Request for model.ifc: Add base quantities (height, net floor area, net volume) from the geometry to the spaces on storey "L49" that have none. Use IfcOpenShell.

First a look at what the model holds.

```python
import ifcopenshell
import ifcopenshell.util.element
import ifcopenshell.util.unit

model = ifcopenshell.open("model.ifc")
print(model.schema)
for unit_type in ("LENGTHUNIT", "AREAUNIT", "VOLUMEUNIT"):
    print(unit_type, ifcopenshell.util.unit.calculate_unit_scale(model, unit_type))
storey = next(s for s in model.by_type("IfcBuildingStorey") if s.Name == "L49")
spaces = [e for e in ifcopenshell.util.element.get_decomposition(storey) if e.is_a("IfcSpace")]
for e in sorted(spaces, key=lambda e: e.id()):
    print(e.id(), e.is_a(), e.Name, list(ifcopenshell.util.element.get_psets(e, qtos_only=True)), sep=" | ")
```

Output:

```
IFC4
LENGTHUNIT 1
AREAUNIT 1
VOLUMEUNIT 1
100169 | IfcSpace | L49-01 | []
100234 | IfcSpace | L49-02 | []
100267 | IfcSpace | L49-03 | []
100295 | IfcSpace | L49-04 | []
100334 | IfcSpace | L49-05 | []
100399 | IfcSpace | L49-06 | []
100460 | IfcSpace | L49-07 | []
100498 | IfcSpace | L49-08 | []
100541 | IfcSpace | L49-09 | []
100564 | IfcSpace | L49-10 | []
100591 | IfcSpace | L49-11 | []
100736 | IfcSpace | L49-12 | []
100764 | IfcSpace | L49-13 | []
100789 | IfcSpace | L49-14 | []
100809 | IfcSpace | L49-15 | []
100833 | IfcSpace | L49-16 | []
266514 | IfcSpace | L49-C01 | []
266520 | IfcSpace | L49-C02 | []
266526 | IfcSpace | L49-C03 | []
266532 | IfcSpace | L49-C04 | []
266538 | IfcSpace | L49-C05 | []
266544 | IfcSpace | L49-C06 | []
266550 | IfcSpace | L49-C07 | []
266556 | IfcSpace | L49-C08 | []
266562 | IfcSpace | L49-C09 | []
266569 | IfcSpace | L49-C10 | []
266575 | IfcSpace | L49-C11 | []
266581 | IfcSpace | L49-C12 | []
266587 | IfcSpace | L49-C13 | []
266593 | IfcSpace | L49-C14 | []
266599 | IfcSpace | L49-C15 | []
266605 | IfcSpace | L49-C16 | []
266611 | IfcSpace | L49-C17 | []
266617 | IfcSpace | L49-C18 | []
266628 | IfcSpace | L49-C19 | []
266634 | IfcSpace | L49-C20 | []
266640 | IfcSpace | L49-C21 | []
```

```python
import ifcopenshell
import ifcopenshell.api.pset
import ifcopenshell.geom
import ifcopenshell.util.element
import ifcopenshell.util.shape
import ifcopenshell.util.unit

model = ifcopenshell.open("model.ifc")
unit_scale = ifcopenshell.util.unit.calculate_unit_scale(model)
area_scale = ifcopenshell.util.unit.calculate_unit_scale(model, "AREAUNIT")
volume_scale = ifcopenshell.util.unit.calculate_unit_scale(model, "VOLUMEUNIT")
settings = ifcopenshell.geom.settings()

storey = next(s for s in model.by_type("IfcBuildingStorey") if s.Name == "L49")
spaces = [e for e in ifcopenshell.util.element.get_decomposition(storey) if e.is_a("IfcSpace")]

for e in sorted(spaces, key=lambda e: e.id()):
    if ifcopenshell.util.element.get_psets(e, qtos_only=True, should_inherit=False):
        continue
    # Geometry comes back in metres, in the element's own axes.
    shape = ifcopenshell.geom.create_shape(settings, e)
    values = {
        "Height": ifcopenshell.util.shape.get_z(shape.geometry) / unit_scale,
        "NetFloorArea": ifcopenshell.util.shape.get_footprint_area(shape.geometry) / area_scale,
        "NetVolume": ifcopenshell.util.shape.get_volume(shape.geometry) / volume_scale,
    }
    qto = ifcopenshell.api.pset.add_qto(model, product=e, name="Qto_SpaceBaseQuantities")
    ifcopenshell.api.pset.edit_qto(model, qto=qto, properties=values)
    print(e.id(), {k: round(v, 3) for k, v in values.items()})

model.write("model-out.ifc")
```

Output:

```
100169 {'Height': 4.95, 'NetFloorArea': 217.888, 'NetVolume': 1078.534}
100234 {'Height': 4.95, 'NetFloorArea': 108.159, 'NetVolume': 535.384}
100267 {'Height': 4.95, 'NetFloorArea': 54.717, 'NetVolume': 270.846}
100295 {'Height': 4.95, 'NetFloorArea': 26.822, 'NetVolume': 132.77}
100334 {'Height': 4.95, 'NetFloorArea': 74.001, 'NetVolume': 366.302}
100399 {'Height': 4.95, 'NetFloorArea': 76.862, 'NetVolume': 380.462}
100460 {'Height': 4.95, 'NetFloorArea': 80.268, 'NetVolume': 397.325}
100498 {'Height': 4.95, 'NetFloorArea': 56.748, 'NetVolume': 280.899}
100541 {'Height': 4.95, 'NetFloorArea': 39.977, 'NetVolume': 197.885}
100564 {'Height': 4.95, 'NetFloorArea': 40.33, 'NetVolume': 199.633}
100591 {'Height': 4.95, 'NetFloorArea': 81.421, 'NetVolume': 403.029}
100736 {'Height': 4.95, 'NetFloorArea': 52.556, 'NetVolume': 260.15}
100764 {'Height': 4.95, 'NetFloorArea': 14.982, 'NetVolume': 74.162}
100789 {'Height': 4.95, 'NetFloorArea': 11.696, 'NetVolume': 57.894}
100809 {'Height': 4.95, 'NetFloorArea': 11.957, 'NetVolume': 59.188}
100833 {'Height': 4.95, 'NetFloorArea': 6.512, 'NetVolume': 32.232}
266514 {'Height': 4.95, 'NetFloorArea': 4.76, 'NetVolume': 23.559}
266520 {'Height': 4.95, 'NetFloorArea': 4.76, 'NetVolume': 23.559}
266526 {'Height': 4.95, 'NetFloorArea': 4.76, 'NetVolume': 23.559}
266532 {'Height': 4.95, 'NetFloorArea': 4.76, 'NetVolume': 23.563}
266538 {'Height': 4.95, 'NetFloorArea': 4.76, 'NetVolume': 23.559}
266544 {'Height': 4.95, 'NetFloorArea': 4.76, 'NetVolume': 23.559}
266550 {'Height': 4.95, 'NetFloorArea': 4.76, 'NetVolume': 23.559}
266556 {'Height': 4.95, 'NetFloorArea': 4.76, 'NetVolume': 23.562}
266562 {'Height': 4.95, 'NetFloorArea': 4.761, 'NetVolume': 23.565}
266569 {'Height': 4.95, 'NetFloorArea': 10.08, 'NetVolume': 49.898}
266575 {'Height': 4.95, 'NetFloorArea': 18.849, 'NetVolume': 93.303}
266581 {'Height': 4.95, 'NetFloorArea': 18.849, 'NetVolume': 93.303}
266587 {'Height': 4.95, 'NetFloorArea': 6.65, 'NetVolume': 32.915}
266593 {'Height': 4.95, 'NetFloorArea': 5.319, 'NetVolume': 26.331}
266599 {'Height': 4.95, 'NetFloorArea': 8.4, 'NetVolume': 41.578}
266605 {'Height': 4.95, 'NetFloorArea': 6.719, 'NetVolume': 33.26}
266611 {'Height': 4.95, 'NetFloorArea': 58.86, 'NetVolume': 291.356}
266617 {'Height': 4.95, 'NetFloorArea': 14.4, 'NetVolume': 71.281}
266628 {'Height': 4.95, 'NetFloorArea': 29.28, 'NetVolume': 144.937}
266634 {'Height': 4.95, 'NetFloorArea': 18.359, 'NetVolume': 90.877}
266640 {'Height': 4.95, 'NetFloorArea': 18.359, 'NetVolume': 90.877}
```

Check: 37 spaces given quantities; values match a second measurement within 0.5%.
